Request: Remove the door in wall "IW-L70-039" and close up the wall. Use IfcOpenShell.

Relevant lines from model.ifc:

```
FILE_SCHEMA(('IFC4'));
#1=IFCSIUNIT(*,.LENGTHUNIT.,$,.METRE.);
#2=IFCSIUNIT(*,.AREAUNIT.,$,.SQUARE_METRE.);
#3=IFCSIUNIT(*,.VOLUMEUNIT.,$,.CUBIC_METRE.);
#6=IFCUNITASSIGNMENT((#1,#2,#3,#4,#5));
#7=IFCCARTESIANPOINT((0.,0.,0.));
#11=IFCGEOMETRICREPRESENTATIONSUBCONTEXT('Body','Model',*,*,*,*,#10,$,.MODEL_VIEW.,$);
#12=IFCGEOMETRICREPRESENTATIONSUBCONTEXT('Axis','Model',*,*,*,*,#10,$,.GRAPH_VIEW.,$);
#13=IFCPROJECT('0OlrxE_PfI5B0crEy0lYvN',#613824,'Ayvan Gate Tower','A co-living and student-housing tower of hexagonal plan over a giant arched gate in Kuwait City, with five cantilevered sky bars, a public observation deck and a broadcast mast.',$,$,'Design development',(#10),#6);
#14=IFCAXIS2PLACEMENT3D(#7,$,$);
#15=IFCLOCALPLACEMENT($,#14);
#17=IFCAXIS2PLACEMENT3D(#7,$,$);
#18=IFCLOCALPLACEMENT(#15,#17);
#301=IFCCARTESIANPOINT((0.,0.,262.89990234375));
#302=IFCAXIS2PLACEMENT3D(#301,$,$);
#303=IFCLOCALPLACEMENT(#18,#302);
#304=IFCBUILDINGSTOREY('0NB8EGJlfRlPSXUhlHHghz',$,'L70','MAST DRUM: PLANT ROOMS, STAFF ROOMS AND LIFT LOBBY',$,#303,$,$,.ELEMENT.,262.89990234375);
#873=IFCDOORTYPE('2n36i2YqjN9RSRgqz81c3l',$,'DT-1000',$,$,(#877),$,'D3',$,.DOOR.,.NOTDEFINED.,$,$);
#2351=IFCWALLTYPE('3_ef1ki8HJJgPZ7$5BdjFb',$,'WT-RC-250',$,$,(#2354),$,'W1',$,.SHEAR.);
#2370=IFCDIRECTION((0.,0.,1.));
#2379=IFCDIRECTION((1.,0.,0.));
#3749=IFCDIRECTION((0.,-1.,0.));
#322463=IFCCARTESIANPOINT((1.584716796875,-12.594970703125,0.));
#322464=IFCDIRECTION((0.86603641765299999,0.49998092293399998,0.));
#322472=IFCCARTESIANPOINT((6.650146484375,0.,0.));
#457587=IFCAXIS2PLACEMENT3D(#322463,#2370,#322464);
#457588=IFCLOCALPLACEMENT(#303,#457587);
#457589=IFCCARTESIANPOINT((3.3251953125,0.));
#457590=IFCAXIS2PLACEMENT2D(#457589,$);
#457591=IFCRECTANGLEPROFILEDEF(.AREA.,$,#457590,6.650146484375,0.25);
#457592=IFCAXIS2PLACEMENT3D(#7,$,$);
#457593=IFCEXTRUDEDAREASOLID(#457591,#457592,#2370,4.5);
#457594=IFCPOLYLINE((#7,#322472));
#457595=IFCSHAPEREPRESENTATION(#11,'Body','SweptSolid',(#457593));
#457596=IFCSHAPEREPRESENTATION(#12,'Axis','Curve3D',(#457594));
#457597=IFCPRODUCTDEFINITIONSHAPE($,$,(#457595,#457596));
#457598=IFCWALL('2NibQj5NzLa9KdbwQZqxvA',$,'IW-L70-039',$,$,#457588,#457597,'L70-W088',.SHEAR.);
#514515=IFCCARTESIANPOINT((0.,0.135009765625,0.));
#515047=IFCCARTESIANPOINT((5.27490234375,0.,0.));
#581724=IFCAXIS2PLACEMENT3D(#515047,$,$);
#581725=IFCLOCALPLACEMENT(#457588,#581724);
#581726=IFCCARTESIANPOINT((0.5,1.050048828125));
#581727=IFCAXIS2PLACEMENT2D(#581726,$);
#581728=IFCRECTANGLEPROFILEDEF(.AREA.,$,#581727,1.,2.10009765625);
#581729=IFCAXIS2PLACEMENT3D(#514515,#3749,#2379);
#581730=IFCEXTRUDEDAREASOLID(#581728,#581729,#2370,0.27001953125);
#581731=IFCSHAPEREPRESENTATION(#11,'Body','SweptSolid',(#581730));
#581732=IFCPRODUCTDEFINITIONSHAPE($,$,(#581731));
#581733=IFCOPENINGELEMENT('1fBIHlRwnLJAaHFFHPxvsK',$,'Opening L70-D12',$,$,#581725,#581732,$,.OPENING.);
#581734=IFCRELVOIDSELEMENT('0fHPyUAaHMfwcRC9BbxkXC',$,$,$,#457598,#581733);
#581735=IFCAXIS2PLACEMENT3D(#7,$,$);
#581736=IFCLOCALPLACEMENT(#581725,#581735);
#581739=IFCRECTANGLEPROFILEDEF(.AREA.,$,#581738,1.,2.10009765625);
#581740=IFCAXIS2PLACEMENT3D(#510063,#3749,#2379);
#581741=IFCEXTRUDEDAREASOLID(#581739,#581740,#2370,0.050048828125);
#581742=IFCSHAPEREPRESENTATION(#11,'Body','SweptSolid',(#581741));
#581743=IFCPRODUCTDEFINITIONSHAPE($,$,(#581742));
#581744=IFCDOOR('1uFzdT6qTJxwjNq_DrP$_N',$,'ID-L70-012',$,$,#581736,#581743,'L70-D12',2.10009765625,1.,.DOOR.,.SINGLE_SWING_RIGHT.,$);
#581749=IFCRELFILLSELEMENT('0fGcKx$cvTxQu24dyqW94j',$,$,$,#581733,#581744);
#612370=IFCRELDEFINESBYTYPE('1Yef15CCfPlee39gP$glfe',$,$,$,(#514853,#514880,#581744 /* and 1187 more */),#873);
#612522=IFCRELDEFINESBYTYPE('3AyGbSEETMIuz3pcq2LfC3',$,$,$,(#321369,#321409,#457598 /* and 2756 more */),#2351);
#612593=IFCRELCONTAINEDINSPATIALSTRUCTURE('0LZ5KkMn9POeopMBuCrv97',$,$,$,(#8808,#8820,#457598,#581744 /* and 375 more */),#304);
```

```python
import ifcopenshell
import ifcopenshell.api.feature
import ifcopenshell.api.root
import ifcopenshell.geom
import ifcopenshell.util.shape

model = ifcopenshell.open("model.ifc")
settings = ifcopenshell.geom.settings()


def volume(element):
    """Net volume in cubic metres, openings subtracted."""
    shape = ifcopenshell.geom.create_shape(settings, element)
    return ifcopenshell.util.shape.get_volume(shape.geometry)


door = model.by_id(581744)
opening = door.FillsVoids[0].RelatingOpeningElement
wall = opening.VoidsElements[0].RelatingBuildingElement
before = volume(wall)

ifcopenshell.api.root.remove_product(model, product=door)
ifcopenshell.api.feature.remove_feature(model, feature=opening)

after = volume(wall)

print(f"wall volume {before:.3f} -> {after:.3f} m3")

model.write("model_edited.ifc")
```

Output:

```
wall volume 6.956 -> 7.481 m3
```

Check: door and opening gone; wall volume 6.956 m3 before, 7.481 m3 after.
